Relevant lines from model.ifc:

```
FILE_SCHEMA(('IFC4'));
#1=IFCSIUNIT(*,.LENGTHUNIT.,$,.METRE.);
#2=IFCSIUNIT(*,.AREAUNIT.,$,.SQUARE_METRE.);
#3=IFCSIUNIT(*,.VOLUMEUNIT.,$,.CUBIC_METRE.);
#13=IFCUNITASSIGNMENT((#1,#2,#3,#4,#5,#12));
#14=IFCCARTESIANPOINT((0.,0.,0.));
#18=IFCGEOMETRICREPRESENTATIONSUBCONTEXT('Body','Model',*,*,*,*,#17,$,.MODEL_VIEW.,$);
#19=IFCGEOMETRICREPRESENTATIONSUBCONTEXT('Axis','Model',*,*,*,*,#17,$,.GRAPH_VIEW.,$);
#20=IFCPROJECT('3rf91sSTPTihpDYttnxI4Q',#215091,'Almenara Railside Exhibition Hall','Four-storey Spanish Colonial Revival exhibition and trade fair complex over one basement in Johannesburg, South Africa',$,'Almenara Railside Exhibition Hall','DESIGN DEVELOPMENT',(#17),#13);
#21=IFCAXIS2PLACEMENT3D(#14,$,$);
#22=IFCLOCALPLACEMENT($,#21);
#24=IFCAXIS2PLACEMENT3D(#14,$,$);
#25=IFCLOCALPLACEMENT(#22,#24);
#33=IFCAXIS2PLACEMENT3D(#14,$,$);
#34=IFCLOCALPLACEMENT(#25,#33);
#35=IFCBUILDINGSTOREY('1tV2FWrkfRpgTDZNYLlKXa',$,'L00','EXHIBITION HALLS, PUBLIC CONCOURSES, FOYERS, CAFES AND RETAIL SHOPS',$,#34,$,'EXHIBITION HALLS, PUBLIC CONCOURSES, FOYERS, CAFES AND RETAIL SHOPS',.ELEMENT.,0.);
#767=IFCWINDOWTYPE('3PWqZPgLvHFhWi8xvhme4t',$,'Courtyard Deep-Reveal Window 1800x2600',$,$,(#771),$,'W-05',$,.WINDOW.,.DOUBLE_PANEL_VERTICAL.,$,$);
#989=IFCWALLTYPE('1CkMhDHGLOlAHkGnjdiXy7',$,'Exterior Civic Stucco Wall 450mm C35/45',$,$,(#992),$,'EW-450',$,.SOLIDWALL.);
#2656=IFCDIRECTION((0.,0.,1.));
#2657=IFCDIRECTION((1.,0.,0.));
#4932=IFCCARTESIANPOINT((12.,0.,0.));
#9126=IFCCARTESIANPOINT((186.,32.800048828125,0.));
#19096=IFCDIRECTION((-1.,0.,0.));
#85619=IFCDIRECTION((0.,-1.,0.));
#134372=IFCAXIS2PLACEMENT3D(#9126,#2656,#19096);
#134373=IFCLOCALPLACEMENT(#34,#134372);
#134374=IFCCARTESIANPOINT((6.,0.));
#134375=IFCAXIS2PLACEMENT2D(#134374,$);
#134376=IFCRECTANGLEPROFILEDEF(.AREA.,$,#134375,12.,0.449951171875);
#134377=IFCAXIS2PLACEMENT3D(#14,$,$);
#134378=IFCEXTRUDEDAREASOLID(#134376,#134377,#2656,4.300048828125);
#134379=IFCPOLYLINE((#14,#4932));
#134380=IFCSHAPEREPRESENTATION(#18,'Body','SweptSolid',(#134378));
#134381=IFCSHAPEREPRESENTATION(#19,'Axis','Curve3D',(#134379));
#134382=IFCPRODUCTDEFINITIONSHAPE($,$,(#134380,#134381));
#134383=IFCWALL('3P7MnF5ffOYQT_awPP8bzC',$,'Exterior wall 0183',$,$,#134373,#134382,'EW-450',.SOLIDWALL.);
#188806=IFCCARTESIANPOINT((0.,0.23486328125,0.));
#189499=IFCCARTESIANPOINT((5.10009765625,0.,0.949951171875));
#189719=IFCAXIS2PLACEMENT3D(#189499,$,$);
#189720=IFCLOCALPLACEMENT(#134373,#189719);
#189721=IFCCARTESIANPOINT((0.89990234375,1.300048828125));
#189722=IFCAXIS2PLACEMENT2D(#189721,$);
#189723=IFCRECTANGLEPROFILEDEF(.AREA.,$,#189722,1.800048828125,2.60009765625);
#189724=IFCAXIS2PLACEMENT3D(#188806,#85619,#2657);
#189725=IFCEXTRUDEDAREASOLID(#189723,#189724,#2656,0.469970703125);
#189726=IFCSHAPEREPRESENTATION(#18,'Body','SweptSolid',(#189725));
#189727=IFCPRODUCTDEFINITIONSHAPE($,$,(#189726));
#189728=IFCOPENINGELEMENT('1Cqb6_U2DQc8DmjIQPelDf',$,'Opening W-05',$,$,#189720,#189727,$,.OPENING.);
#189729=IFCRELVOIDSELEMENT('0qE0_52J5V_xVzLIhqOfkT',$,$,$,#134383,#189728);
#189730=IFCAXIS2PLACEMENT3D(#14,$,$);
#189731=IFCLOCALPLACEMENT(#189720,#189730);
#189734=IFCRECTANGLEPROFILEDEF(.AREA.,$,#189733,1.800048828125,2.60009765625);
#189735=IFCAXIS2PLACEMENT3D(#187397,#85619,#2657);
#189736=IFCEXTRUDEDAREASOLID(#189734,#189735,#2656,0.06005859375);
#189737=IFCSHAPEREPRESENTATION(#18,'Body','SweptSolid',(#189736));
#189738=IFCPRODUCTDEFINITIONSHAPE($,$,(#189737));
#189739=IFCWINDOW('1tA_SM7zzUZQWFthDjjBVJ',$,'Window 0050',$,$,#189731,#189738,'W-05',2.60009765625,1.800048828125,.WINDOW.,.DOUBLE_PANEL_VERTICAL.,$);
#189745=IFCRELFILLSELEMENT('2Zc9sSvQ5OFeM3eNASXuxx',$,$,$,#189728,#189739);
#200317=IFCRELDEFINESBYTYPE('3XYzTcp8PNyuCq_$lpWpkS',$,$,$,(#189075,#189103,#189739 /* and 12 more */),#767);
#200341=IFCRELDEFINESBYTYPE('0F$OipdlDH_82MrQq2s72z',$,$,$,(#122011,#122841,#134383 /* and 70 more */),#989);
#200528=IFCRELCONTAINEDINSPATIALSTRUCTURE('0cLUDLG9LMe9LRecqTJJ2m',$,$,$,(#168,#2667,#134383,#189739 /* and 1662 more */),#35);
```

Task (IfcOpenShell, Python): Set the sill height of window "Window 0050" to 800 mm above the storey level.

```python
import numpy as np
import ifcopenshell
import ifcopenshell.api.geometry
import ifcopenshell.geom
import ifcopenshell.util.element
import ifcopenshell.util.placement
import ifcopenshell.util.shape
import ifcopenshell.util.unit

model = ifcopenshell.open("model.ifc")
unit_scale = ifcopenshell.util.unit.calculate_unit_scale(model)

window = model.by_guid("1tA_SM7zzUZQWFthDjjBVJ")
opening = window.FillsVoids[0].RelatingOpeningElement
storey = ifcopenshell.util.element.get_container(window, ifc_class="IfcBuildingStorey")
level = ifcopenshell.util.placement.get_local_placement(storey.ObjectPlacement)[2, 3]

# The opening's origin need not be at the sill, so measure its lowest point.
shape = ifcopenshell.geom.create_shape(ifcopenshell.geom.settings(), opening)
bottom = ifcopenshell.util.shape.get_shape_bottom_elevation(shape, shape.geometry) / unit_scale
dz = level + 0.8 - bottom

shift = np.array([0.0, 0.0, dz])
# The window is placed relative to its opening, so it follows when the opening moves.
matrix = ifcopenshell.util.placement.get_local_placement(opening.ObjectPlacement)
matrix[:3, 3] += shift
ifcopenshell.api.geometry.edit_object_placement(
    model, product=opening, matrix=matrix, is_si=False, should_transform_children=True
)

print(f"moved by {dz * unit_scale:+.3f} m")

model.write("model_v2.ifc")
```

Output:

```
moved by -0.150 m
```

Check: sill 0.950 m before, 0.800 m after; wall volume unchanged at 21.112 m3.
